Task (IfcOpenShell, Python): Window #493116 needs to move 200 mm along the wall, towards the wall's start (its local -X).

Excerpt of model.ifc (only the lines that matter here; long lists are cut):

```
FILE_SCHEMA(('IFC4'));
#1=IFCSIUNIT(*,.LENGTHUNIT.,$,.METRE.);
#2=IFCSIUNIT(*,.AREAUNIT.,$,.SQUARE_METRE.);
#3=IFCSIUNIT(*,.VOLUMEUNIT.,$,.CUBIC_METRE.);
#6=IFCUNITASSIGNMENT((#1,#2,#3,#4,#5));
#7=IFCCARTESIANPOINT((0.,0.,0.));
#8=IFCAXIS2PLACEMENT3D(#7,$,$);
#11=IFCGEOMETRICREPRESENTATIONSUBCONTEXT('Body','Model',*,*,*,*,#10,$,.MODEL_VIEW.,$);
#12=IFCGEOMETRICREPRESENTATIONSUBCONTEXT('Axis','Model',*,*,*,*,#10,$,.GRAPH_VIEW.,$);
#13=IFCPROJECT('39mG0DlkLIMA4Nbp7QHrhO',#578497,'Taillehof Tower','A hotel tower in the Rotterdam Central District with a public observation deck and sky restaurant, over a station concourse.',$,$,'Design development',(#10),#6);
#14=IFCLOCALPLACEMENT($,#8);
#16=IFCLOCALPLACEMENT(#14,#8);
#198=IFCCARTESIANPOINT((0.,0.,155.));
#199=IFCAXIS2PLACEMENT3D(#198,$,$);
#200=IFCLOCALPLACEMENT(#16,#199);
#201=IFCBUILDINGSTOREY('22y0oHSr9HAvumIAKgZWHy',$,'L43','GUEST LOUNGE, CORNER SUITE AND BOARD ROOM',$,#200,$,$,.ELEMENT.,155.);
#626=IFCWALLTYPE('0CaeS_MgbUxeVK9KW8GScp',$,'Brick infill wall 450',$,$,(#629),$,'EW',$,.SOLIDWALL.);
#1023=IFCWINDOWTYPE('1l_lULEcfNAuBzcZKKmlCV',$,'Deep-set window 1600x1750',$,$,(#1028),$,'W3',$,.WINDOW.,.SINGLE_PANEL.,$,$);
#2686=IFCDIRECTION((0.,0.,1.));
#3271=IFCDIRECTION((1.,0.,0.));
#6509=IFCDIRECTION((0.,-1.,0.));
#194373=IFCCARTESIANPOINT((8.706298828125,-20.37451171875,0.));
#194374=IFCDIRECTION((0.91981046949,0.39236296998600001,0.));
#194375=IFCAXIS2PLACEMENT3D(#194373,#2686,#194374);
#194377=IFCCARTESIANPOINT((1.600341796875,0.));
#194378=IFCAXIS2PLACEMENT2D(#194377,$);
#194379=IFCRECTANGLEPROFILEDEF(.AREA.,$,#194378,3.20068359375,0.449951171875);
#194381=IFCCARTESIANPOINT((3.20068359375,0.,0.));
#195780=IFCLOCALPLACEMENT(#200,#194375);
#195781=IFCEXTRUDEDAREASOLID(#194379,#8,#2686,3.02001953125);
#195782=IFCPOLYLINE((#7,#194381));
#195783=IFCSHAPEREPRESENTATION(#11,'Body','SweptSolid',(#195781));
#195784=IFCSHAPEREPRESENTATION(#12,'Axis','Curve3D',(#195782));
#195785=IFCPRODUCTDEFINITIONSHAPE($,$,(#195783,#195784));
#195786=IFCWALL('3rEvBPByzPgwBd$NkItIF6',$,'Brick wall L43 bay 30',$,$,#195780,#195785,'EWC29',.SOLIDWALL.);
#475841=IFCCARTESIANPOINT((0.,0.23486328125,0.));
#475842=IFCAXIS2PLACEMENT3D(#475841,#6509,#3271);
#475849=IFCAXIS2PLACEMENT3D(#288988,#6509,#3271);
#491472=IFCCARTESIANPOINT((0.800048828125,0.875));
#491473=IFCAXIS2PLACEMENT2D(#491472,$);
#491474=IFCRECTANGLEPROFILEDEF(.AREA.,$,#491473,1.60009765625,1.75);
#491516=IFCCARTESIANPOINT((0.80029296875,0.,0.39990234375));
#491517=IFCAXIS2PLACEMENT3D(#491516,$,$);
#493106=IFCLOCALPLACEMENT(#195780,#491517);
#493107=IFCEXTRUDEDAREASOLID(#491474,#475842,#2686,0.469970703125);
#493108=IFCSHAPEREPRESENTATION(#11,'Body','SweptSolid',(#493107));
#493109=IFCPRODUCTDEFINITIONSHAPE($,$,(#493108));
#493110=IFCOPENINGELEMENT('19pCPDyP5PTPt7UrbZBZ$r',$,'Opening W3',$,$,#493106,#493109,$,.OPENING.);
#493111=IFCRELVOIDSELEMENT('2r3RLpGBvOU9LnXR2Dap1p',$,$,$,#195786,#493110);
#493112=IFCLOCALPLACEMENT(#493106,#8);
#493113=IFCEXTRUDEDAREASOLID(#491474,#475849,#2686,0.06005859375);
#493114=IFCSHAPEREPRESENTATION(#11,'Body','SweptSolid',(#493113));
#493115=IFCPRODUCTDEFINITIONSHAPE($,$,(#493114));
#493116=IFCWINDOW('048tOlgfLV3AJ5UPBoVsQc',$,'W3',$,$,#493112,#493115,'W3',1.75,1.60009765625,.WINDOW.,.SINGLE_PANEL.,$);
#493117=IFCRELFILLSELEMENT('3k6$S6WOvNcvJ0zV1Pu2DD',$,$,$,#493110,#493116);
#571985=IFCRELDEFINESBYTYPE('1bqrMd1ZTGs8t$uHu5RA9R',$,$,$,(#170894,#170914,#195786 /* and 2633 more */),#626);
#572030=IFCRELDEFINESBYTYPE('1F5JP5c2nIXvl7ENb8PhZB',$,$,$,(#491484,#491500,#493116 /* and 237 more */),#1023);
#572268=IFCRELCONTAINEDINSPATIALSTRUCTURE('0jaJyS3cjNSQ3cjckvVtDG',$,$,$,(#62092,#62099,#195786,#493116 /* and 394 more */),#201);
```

```python
import ifcopenshell
import ifcopenshell.api.geometry
import ifcopenshell.util.placement
import ifcopenshell.util.unit

model = ifcopenshell.open("model.ifc")
unit_scale = ifcopenshell.util.unit.calculate_unit_scale(model)

window = model.by_guid("048tOlgfLV3AJ5UPBoVsQc")
opening = window.FillsVoids[0].RelatingOpeningElement
wall = opening.VoidsElements[0].RelatingBuildingElement

wall_matrix = ifcopenshell.util.placement.get_local_placement(wall.ObjectPlacement)
shift = wall_matrix[:3, 0] * -0.2 / unit_scale
before = ifcopenshell.util.placement.get_local_placement(window.ObjectPlacement)[:3, 3].copy()

# The window is placed relative to its opening, so it follows when the opening moves.
matrix = ifcopenshell.util.placement.get_local_placement(opening.ObjectPlacement)
matrix[:3, 3] += shift
ifcopenshell.api.geometry.edit_object_placement(
    model, product=opening, matrix=matrix, is_si=False, should_transform_children=True
)

after = ifcopenshell.util.placement.get_local_placement(window.ObjectPlacement)[:3, 3]
print("window moved by", (after - before).round(3) + 0.0)

model.write("model-out.ifc")
```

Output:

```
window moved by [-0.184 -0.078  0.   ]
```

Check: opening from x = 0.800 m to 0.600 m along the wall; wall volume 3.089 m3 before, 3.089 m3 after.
